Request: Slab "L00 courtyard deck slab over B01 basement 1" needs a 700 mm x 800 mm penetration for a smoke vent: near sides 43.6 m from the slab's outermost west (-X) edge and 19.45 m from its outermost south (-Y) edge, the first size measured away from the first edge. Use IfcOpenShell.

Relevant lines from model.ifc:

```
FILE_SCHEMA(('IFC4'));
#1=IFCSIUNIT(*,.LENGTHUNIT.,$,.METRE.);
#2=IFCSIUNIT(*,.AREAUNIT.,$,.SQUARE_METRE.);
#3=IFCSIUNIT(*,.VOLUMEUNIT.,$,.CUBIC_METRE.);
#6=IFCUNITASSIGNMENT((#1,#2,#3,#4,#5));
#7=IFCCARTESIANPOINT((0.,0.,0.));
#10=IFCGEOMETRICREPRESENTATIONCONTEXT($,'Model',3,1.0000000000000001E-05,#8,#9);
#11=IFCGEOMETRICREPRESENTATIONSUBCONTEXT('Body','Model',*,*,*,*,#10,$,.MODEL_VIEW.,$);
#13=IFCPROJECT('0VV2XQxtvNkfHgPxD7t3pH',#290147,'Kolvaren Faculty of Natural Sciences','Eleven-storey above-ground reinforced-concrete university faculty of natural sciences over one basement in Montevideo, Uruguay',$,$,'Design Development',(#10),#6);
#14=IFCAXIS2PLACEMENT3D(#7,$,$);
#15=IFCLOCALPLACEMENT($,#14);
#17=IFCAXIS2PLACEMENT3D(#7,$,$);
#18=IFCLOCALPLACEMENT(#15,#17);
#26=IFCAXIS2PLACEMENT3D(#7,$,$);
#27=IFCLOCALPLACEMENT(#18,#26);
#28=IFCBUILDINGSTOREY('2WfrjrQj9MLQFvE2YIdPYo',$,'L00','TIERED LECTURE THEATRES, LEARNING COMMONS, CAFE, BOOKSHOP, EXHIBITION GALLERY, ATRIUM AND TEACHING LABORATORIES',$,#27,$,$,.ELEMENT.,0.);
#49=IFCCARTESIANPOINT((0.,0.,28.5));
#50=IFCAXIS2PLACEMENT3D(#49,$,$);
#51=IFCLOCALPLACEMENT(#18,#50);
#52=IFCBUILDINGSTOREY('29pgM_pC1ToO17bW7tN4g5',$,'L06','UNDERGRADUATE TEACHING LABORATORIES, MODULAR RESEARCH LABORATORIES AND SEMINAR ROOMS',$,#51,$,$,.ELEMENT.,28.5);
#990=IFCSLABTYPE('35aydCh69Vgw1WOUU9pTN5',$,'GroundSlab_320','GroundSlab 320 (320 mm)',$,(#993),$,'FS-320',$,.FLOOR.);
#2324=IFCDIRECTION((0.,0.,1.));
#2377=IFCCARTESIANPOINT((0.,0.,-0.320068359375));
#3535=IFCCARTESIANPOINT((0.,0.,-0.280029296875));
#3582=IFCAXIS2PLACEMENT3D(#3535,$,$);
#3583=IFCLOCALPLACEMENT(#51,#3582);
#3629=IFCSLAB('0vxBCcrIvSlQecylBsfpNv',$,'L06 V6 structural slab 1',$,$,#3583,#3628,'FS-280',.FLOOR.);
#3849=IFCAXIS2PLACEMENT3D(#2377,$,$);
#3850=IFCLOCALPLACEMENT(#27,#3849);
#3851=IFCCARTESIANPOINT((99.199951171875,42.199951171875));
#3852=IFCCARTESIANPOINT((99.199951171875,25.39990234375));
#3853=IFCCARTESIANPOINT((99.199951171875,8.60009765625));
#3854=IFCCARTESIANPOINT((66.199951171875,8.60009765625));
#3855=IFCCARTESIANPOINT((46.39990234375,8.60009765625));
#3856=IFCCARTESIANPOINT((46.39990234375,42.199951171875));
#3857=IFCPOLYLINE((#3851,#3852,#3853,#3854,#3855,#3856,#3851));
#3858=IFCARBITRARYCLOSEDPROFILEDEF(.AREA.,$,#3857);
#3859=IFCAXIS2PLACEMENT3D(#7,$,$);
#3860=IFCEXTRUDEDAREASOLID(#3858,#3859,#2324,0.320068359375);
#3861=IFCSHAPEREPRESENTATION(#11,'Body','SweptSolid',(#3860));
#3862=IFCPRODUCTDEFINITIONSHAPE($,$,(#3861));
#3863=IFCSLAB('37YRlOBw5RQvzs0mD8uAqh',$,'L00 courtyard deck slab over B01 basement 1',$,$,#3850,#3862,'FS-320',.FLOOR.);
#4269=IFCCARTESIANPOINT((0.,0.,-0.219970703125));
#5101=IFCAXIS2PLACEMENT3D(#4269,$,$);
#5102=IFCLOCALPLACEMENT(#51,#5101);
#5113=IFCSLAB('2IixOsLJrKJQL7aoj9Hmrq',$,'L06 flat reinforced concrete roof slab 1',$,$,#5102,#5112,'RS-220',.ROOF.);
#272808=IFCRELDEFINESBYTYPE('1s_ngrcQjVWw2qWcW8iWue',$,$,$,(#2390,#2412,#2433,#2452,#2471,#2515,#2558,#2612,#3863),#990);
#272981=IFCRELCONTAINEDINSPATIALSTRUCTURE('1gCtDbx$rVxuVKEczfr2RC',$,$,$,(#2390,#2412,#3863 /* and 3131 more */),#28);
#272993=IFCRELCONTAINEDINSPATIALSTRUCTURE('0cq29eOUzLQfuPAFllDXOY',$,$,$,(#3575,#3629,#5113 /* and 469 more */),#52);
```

```python
import numpy as np
import ifcopenshell
import ifcopenshell.api.feature
import ifcopenshell.api.geometry
import ifcopenshell.api.root
import ifcopenshell.geom
import ifcopenshell.util.placement
import ifcopenshell.util.representation
import ifcopenshell.util.shape
import ifcopenshell.util.unit

model = ifcopenshell.open("model.ifc")
unit_scale = ifcopenshell.util.unit.calculate_unit_scale(model)
settings = ifcopenshell.geom.settings()


def volume(element):
    """Net volume in cubic metres, openings subtracted."""
    shape = ifcopenshell.geom.create_shape(settings, element)
    return ifcopenshell.util.shape.get_volume(shape.geometry)


slab = model.by_id(3863)
before = volume(slab)

# Extent in the slab's own axes, in metres. The edges named are its -X and -Y sides.
slab_shape = ifcopenshell.geom.create_shape(settings, slab)
vertices = ifcopenshell.util.shape.get_vertices(slab_shape.geometry)
x_min, y_min, bottom = vertices.min(axis=0)
top = vertices[:, 2].max()

opening = ifcopenshell.api.root.create_entity(model, ifc_class="IfcOpeningElement", name="Smoke vent opening", predefined_type="OPENING")
context = ifcopenshell.util.representation.get_context(model, "Model", "Body", "MODEL_VIEW")
width, depth = 0.7, 0.8
outline = [(0.0, 0.0), (width, 0.0), (width, depth), (0.0, depth), (0.0, 0.0)]
# Overshoot both faces by 50 mm so the cut is clean.
shape = ifcopenshell.api.geometry.add_slab_representation(
    model, context=context, depth=top - bottom + 0.1, polyline=outline
)
ifcopenshell.api.geometry.assign_representation(model, product=opening, representation=shape)

matrix = ifcopenshell.util.placement.get_local_placement(slab.ObjectPlacement)
matrix[:, 3] = matrix @ np.append(np.array([x_min + 43.6, y_min + 19.45, bottom - 0.05]) / unit_scale, 1.0)
ifcopenshell.api.geometry.edit_object_placement(model, product=opening, matrix=matrix, is_si=False)
ifcopenshell.api.feature.add_feature(model, feature=opening, element=slab)

after = volume(slab)

print(f"slab volume {before:.3f} -> {after:.3f} m3")

model.write("model_updated.ifc")
```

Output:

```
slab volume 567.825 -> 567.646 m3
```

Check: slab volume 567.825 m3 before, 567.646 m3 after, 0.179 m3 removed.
